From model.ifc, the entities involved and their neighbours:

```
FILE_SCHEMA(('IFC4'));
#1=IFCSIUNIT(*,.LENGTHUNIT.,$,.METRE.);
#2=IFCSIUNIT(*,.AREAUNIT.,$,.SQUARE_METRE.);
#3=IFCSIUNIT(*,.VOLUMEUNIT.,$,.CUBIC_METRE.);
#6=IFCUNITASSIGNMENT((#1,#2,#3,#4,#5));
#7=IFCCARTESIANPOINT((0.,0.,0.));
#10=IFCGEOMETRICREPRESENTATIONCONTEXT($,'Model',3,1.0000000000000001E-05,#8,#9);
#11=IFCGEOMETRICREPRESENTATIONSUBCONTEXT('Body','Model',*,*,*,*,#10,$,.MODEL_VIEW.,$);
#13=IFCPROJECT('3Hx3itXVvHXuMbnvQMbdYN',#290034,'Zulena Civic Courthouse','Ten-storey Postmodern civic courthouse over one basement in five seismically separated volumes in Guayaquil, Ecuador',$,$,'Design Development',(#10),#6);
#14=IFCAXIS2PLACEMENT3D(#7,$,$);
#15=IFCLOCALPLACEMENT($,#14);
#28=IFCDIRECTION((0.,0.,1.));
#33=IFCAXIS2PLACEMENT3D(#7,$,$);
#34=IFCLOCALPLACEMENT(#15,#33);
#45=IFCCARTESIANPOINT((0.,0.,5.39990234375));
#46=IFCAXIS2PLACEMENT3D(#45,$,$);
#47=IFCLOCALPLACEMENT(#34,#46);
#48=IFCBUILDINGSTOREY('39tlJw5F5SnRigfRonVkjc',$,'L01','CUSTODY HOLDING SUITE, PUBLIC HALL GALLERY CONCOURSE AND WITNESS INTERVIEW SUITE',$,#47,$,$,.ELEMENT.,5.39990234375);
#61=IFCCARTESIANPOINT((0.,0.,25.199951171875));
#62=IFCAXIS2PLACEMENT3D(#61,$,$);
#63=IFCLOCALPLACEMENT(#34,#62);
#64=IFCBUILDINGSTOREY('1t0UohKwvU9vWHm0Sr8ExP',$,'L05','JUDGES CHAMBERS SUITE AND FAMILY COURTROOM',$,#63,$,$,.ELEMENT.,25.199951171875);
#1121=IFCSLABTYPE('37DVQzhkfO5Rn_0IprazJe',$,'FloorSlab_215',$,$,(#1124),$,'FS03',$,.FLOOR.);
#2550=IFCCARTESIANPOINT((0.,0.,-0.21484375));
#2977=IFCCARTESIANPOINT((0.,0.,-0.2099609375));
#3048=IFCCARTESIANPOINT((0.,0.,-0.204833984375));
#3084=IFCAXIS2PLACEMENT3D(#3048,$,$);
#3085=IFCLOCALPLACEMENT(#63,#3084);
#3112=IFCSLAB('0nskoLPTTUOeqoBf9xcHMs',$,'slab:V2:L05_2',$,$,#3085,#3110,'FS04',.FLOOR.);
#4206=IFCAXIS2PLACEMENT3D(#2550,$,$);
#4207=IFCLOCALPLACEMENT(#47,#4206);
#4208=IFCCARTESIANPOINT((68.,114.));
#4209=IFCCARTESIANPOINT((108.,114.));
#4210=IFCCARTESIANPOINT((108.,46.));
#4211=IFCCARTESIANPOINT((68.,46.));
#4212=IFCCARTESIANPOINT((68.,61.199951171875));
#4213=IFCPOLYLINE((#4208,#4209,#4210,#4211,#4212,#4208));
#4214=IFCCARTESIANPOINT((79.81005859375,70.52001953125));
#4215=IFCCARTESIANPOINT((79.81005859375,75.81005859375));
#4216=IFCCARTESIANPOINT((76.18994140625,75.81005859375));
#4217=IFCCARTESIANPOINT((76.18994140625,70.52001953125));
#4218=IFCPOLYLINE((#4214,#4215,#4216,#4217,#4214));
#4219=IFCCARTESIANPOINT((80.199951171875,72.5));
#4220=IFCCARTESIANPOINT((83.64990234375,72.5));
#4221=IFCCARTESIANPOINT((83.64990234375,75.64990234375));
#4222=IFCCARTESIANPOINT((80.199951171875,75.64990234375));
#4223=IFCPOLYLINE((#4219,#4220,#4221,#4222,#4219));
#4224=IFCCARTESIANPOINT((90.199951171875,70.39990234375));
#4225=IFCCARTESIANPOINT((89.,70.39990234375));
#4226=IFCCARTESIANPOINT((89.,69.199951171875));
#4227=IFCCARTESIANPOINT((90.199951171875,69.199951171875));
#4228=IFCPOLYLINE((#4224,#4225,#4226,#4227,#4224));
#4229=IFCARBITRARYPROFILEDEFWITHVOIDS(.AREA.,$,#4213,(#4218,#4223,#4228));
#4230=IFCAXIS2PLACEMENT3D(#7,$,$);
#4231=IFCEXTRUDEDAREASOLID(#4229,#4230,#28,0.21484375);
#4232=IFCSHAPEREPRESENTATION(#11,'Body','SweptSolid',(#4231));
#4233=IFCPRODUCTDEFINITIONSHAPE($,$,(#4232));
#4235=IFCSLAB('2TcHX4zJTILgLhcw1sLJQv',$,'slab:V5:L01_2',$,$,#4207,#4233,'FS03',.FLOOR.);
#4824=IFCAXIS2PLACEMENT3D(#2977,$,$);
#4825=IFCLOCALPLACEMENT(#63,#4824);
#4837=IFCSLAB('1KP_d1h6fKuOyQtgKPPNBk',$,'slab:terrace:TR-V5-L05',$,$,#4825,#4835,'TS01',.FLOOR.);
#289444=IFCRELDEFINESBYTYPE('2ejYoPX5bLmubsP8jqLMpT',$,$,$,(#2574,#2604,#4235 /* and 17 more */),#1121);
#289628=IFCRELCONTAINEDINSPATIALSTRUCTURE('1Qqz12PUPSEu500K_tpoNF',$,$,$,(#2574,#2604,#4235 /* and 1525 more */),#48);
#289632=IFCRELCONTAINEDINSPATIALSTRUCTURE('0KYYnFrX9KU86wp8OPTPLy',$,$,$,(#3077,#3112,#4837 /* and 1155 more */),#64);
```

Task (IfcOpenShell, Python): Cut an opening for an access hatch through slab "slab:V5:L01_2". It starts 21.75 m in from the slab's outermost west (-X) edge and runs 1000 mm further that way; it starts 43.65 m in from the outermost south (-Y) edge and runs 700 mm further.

```python
import numpy as np
import ifcopenshell
import ifcopenshell.api.feature
import ifcopenshell.api.geometry
import ifcopenshell.api.root
import ifcopenshell.geom
import ifcopenshell.util.placement
import ifcopenshell.util.representation
import ifcopenshell.util.shape
import ifcopenshell.util.unit

model = ifcopenshell.open("model.ifc")
unit_scale = ifcopenshell.util.unit.calculate_unit_scale(model)
settings = ifcopenshell.geom.settings()


def volume(element):
    """Net volume in cubic metres, openings subtracted."""
    shape = ifcopenshell.geom.create_shape(settings, element)
    return ifcopenshell.util.shape.get_volume(shape.geometry)


slab = model.by_id(4235)
before = volume(slab)

# Extent in the slab's own axes, in metres. The edges named are its -X and -Y sides.
slab_shape = ifcopenshell.geom.create_shape(settings, slab)
vertices = ifcopenshell.util.shape.get_vertices(slab_shape.geometry)
x_min, y_min, bottom = vertices.min(axis=0)
top = vertices[:, 2].max()

opening = ifcopenshell.api.root.create_entity(model, ifc_class="IfcOpeningElement", name="Access hatch opening", predefined_type="OPENING")
context = ifcopenshell.util.representation.get_context(model, "Model", "Body", "MODEL_VIEW")
width, depth = 1, 0.7
outline = [(0.0, 0.0), (width, 0.0), (width, depth), (0.0, depth), (0.0, 0.0)]
# Overshoot both faces by 50 mm so the cut is clean.
shape = ifcopenshell.api.geometry.add_slab_representation(
    model, context=context, depth=top - bottom + 0.1, polyline=outline
)
ifcopenshell.api.geometry.assign_representation(model, product=opening, representation=shape)

matrix = ifcopenshell.util.placement.get_local_placement(slab.ObjectPlacement)
matrix[:, 3] = matrix @ np.append(np.array([x_min + 21.75, y_min + 43.65, bottom - 0.05]) / unit_scale, 1.0)
ifcopenshell.api.geometry.edit_object_placement(model, product=opening, matrix=matrix, is_si=False)
ifcopenshell.api.feature.add_feature(model, feature=opening, element=slab)

after = volume(slab)

print(f"slab volume {before:.3f} -> {after:.3f} m3")

model.write("model_updated.ifc")
```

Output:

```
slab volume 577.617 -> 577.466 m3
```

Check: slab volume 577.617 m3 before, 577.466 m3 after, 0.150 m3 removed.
